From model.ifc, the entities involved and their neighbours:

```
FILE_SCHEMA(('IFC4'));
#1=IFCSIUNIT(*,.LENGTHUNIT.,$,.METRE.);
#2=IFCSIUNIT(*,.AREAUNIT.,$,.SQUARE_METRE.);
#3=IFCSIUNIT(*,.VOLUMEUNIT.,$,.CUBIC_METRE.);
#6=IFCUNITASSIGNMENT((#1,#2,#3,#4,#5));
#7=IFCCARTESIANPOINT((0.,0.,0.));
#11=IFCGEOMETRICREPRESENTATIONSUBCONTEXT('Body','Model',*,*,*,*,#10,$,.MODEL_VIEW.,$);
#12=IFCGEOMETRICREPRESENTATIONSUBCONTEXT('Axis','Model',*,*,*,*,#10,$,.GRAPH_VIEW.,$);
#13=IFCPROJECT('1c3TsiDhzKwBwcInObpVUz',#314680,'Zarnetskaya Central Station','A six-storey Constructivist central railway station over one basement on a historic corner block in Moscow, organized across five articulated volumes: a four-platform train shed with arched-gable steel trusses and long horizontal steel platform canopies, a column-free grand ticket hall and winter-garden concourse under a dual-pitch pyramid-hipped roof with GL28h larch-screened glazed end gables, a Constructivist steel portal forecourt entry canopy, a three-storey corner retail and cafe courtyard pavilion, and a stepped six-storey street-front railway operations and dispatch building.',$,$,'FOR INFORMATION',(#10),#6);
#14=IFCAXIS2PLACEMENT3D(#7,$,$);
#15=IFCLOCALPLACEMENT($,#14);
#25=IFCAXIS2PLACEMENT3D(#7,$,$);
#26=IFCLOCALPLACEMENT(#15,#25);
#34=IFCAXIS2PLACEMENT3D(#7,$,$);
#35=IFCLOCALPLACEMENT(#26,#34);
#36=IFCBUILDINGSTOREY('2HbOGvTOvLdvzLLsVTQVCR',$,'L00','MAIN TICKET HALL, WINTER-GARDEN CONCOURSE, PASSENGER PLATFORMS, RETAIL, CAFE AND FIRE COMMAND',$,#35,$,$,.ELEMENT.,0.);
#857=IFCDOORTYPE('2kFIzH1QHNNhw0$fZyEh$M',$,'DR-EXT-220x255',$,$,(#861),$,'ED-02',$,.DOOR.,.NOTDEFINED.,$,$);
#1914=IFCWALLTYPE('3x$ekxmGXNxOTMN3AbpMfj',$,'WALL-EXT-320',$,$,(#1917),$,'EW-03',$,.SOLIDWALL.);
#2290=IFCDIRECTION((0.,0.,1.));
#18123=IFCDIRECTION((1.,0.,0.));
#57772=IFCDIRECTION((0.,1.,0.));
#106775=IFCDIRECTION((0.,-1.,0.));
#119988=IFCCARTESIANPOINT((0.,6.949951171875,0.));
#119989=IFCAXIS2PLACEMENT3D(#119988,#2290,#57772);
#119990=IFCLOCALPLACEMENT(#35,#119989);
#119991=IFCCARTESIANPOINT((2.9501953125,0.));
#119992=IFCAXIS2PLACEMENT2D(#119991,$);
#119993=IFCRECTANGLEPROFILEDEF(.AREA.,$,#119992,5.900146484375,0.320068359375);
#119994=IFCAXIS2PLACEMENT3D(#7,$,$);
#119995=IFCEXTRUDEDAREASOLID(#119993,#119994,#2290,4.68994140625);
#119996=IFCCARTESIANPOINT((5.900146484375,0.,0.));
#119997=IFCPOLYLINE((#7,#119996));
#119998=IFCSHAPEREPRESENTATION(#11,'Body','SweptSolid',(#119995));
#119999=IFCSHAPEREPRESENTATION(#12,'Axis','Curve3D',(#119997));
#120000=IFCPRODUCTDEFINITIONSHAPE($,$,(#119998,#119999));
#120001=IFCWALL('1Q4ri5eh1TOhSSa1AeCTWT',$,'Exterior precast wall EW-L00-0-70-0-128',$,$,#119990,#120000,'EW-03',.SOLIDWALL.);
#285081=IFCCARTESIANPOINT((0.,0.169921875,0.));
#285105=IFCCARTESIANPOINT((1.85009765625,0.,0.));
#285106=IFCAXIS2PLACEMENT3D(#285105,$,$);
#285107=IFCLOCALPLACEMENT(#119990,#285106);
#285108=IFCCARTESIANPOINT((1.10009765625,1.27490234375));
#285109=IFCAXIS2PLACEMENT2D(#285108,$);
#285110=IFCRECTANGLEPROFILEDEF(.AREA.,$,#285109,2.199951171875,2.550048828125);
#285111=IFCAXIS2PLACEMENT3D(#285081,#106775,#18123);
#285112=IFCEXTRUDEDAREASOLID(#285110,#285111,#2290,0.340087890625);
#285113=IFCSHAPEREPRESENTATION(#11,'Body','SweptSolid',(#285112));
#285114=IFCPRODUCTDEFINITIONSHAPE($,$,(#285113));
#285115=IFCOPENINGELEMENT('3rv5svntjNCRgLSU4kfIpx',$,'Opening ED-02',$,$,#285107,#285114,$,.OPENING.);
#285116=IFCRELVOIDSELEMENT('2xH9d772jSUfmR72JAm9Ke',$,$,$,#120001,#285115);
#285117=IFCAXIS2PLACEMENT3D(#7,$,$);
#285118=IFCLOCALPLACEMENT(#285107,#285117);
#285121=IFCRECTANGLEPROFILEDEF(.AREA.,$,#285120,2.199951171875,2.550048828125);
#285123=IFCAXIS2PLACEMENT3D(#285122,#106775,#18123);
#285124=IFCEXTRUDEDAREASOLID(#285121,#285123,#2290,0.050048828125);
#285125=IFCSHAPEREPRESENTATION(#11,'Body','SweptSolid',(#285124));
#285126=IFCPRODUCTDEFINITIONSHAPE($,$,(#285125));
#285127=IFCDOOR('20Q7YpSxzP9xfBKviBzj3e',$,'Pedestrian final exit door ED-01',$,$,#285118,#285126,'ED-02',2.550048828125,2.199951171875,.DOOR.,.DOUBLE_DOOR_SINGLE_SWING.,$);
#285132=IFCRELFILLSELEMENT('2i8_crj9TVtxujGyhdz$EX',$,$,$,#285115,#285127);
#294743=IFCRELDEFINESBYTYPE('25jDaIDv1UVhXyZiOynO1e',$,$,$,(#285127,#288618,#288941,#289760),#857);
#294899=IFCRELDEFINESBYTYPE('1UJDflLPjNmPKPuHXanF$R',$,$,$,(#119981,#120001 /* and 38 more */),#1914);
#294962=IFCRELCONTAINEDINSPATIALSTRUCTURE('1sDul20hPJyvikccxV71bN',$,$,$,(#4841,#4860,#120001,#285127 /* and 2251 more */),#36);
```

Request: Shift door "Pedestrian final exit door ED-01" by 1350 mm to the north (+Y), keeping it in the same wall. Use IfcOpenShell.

```python
import ifcopenshell
import ifcopenshell.api.geometry
import ifcopenshell.util.placement
import ifcopenshell.util.unit

model = ifcopenshell.open("model.ifc")
unit_scale = ifcopenshell.util.unit.calculate_unit_scale(model)

door = model.by_guid("20Q7YpSxzP9xfBKviBzj3e")
opening = door.FillsVoids[0].RelatingOpeningElement
wall = opening.VoidsElements[0].RelatingBuildingElement

wall_matrix = ifcopenshell.util.placement.get_local_placement(wall.ObjectPlacement)
shift = wall_matrix[:3, 0] * 1.35 / unit_scale
before = ifcopenshell.util.placement.get_local_placement(door.ObjectPlacement)[:3, 3].copy()

# The door is placed relative to its opening, so it follows when the opening moves.
matrix = ifcopenshell.util.placement.get_local_placement(opening.ObjectPlacement)
matrix[:3, 3] += shift
ifcopenshell.api.geometry.edit_object_placement(
    model, product=opening, matrix=matrix, is_si=False, should_transform_children=True
)

after = ifcopenshell.util.placement.get_local_placement(door.ObjectPlacement)[:3, 3]
print("door moved by", (after - before).round(3) + 0.0)

model.write("model_rev.ifc")
```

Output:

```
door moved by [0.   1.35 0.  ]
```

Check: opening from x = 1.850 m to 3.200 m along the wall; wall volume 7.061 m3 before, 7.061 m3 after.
